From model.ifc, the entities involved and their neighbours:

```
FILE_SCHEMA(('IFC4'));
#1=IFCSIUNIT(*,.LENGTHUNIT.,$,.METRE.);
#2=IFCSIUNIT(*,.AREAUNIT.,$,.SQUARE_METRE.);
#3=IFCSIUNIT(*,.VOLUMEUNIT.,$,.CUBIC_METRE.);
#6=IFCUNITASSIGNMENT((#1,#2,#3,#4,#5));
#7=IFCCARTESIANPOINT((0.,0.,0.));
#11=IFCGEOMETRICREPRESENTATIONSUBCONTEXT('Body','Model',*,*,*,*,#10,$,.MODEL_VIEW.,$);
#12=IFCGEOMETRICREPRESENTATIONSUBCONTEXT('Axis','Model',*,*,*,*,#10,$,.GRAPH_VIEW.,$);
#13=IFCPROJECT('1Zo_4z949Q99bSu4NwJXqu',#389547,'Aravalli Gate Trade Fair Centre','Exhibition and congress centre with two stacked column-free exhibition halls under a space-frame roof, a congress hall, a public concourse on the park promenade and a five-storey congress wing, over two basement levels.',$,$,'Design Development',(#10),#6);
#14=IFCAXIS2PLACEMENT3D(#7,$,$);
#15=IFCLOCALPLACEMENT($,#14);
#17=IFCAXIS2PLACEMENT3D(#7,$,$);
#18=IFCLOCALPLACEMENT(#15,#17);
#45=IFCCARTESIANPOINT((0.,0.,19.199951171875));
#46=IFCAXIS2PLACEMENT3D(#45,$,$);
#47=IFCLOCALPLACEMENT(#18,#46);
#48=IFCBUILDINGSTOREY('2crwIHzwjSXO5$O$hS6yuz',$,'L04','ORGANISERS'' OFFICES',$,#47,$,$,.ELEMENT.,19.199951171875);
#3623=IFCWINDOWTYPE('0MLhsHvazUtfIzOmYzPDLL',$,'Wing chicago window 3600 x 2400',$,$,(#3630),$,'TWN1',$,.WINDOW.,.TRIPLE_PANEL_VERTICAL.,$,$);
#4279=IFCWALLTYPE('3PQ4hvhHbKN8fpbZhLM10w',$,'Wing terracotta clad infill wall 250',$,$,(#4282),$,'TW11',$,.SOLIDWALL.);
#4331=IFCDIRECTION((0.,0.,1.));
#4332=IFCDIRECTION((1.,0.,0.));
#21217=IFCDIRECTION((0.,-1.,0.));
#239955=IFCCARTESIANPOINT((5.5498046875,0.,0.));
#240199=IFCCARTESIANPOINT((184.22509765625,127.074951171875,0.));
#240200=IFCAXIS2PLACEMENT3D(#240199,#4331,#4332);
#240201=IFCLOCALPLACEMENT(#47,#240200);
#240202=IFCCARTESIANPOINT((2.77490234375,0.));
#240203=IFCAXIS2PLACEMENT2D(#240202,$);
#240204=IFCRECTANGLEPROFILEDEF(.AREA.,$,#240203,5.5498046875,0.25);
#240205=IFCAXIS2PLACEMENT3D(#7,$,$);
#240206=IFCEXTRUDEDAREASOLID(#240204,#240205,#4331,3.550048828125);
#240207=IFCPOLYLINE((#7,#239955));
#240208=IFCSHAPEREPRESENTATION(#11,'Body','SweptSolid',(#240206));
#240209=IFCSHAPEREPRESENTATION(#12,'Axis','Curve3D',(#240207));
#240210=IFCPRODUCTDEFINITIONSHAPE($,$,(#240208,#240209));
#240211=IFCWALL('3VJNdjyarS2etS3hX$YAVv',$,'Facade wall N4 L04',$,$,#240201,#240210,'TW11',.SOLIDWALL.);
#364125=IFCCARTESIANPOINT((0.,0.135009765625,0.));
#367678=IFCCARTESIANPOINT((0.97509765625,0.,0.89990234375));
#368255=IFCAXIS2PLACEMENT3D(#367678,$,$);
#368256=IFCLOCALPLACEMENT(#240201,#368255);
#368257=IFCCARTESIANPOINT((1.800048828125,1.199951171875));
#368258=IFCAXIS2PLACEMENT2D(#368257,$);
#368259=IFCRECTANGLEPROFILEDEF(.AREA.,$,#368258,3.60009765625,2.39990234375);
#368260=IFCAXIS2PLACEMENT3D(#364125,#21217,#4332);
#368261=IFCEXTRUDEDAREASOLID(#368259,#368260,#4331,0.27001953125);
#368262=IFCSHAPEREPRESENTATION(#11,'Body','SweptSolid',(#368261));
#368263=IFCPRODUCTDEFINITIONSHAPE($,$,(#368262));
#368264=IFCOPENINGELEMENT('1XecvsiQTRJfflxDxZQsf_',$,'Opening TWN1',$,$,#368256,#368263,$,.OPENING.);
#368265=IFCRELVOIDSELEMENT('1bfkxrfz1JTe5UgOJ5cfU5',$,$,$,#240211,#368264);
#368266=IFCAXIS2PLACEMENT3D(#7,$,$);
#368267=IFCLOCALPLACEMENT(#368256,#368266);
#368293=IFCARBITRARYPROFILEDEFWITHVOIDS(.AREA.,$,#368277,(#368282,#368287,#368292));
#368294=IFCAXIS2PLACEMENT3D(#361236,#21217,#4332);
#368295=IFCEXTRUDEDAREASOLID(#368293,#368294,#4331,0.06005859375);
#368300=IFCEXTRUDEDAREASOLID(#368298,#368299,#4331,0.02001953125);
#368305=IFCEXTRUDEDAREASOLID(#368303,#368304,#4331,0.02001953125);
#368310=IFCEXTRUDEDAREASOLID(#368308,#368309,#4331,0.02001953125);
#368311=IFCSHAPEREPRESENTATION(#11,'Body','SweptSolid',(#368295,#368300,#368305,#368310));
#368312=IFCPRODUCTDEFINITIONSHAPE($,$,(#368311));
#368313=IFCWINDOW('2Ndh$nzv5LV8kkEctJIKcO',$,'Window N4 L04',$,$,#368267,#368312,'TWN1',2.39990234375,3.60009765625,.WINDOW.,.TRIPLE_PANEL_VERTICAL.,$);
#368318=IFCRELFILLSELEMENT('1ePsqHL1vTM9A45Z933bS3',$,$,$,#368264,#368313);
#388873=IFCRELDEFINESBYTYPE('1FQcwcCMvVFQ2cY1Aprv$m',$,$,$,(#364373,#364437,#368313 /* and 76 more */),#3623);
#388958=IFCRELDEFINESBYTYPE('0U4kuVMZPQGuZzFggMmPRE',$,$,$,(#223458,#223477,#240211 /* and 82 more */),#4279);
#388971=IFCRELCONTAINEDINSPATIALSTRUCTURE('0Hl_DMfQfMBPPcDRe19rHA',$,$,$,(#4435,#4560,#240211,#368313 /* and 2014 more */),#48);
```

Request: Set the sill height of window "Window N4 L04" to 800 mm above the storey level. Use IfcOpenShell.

```python
import numpy as np
import ifcopenshell
import ifcopenshell.api.geometry
import ifcopenshell.geom
import ifcopenshell.util.element
import ifcopenshell.util.placement
import ifcopenshell.util.shape
import ifcopenshell.util.unit

model = ifcopenshell.open("model.ifc")
unit_scale = ifcopenshell.util.unit.calculate_unit_scale(model)

window = model.by_guid("2Ndh$nzv5LV8kkEctJIKcO")
opening = window.FillsVoids[0].RelatingOpeningElement
storey = ifcopenshell.util.element.get_container(window, ifc_class="IfcBuildingStorey")
level = ifcopenshell.util.placement.get_local_placement(storey.ObjectPlacement)[2, 3]

# The opening's origin need not be at the sill, so measure its lowest point.
shape = ifcopenshell.geom.create_shape(ifcopenshell.geom.settings(), opening)
bottom = ifcopenshell.util.shape.get_shape_bottom_elevation(shape, shape.geometry) / unit_scale
dz = level + 0.8 / unit_scale - bottom

shift = np.array([0.0, 0.0, dz])
# The window is placed relative to its opening, so it follows when the opening moves.
matrix = ifcopenshell.util.placement.get_local_placement(opening.ObjectPlacement)
matrix[:3, 3] += shift
ifcopenshell.api.geometry.edit_object_placement(
    model, product=opening, matrix=matrix, is_si=False, should_transform_children=True
)

print(f"moved by {dz * unit_scale:+.3f} m")

model.write("model_edited.ifc")
```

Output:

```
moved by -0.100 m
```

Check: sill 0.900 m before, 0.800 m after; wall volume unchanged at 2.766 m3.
